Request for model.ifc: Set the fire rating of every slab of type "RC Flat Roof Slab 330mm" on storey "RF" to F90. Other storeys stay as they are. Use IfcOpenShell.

First a look at what the model holds.

```python
import ifcopenshell
import ifcopenshell.util.element

model = ifcopenshell.open("model.ifc")
print(model.schema)
storey = next(s for s in model.by_type("IfcBuildingStorey") if s.Name == "RF")
slabs = [e for e in ifcopenshell.util.element.get_decomposition(storey) if e.is_a("IfcSlab")]
seen = {}
for e in slabs:
    element_type = ifcopenshell.util.element.get_type(e)
    key = (element_type.Name if element_type != e and element_type else None, ifcopenshell.util.element.get_pset(e, "Pset_SlabCommon", "FireRating"))
    seen[key] = seen.get(key, 0) + 1
for (name, value), count in sorted(seen.items(), key=str):
    print(count, "x", name, "|", value)
```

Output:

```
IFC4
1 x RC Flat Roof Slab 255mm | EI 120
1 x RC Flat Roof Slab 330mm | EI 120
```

```python
import ifcopenshell
import ifcopenshell.api.pset
import ifcopenshell.util.element

model = ifcopenshell.open("model.ifc")

storey = next(s for s in model.by_type("IfcBuildingStorey") if s.Name == "RF")
slabs = [e for e in ifcopenshell.util.element.get_decomposition(storey) if e.is_a("IfcSlab")]

count = 0
for e in slabs:
    element_type = ifcopenshell.util.element.get_type(e)
    if element_type in (None, e) or element_type.Name != "RC Flat Roof Slab 330mm":
        continue
    # add_pset returns the element's existing set when there is one.
    pset = ifcopenshell.api.pset.add_pset(model, product=e, name="Pset_SlabCommon")
    ifcopenshell.api.pset.edit_pset(model, pset=pset, properties={"FireRating": "F90"})
    count += 1

print(count, "slabs updated")

model.write("model_updated.ifc")
```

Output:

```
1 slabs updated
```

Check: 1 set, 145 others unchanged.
